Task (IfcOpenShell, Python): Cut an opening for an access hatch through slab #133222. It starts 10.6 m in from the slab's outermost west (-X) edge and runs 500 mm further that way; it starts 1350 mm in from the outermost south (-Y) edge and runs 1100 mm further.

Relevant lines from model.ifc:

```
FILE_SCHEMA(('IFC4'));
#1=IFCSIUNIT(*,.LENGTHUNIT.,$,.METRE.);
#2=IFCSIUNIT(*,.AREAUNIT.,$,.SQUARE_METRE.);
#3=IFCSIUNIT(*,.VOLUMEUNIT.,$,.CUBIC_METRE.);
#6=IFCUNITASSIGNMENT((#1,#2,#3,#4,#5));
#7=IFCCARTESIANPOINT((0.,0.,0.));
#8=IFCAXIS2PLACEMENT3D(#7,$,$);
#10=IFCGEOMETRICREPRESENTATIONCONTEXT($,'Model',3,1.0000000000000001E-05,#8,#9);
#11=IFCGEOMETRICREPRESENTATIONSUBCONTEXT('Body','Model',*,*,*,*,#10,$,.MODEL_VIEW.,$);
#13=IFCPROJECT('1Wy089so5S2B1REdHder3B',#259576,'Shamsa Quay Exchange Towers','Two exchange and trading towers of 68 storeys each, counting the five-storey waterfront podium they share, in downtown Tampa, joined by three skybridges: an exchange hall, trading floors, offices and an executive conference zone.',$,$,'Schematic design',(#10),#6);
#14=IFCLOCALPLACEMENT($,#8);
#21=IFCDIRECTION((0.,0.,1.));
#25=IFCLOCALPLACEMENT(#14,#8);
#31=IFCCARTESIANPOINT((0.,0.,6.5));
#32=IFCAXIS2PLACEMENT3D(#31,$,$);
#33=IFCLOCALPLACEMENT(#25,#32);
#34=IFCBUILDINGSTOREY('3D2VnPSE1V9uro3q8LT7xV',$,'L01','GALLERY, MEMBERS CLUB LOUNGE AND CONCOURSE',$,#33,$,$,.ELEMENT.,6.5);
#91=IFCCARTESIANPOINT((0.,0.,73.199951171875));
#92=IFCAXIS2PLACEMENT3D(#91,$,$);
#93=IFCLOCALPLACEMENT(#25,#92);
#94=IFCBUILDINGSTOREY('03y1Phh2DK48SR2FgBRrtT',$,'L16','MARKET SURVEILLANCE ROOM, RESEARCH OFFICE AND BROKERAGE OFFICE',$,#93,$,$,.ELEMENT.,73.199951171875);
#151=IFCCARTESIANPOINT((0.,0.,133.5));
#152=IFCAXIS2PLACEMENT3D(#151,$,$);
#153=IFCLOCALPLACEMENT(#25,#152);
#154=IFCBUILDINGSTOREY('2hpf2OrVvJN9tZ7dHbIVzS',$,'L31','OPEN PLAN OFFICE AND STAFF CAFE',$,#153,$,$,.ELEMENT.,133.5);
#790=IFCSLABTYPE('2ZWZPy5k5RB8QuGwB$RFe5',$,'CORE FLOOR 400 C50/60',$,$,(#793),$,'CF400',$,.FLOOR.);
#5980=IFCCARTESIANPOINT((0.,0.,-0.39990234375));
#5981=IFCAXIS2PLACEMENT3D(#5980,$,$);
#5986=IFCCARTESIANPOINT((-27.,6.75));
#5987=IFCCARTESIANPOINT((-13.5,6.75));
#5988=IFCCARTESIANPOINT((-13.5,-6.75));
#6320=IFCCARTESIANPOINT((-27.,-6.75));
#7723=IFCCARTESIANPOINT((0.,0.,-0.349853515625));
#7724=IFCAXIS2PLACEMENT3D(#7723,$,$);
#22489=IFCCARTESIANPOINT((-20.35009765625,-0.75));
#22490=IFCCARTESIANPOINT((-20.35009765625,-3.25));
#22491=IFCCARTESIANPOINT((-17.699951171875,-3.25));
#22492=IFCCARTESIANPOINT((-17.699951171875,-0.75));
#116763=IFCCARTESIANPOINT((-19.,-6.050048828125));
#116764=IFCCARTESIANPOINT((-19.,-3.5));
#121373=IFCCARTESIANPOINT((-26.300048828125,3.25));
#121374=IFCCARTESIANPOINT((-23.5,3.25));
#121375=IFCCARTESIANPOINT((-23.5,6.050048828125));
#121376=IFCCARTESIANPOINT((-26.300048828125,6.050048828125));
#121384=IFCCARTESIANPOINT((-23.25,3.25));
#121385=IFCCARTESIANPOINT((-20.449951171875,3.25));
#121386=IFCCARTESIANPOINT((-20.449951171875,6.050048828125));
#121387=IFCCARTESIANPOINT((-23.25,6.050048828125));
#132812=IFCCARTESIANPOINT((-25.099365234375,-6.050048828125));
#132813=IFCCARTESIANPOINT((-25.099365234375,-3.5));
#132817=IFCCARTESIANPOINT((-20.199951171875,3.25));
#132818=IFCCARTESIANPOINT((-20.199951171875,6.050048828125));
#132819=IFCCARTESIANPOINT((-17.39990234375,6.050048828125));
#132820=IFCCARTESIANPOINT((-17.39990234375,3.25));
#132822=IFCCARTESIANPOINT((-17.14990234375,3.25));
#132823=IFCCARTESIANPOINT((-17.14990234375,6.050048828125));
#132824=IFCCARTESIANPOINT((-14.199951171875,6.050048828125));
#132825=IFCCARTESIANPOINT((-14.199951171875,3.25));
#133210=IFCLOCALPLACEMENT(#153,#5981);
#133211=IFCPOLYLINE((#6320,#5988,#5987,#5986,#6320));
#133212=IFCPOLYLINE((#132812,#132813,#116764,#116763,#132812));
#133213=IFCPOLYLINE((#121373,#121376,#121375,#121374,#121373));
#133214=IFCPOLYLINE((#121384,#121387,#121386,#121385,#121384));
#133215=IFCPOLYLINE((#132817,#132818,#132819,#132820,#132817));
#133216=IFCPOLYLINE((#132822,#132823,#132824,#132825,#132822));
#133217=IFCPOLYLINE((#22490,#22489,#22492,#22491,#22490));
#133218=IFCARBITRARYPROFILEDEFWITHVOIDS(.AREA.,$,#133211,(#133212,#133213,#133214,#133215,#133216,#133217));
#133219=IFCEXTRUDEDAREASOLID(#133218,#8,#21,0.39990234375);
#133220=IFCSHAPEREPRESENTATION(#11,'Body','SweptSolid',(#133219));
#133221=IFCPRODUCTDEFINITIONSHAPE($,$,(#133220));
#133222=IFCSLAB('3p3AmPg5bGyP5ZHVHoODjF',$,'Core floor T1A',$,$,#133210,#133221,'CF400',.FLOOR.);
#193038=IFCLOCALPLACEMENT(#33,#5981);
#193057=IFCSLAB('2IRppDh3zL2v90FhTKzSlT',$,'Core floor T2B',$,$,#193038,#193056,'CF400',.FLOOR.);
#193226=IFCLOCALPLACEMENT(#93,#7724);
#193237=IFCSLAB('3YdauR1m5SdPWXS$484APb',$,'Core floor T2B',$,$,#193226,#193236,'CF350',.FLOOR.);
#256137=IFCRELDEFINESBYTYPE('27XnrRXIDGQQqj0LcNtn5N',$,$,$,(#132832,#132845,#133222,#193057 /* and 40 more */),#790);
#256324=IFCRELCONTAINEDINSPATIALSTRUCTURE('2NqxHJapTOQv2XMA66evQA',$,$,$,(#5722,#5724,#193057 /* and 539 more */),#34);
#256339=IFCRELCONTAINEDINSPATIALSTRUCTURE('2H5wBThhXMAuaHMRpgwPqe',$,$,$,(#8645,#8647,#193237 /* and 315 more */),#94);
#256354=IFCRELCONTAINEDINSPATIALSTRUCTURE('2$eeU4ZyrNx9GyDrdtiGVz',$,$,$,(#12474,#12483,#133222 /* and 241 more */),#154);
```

```python
import numpy as np
import ifcopenshell
import ifcopenshell.api.feature
import ifcopenshell.api.geometry
import ifcopenshell.api.root
import ifcopenshell.geom
import ifcopenshell.util.placement
import ifcopenshell.util.representation
import ifcopenshell.util.shape
import ifcopenshell.util.unit

model = ifcopenshell.open("model.ifc")
unit_scale = ifcopenshell.util.unit.calculate_unit_scale(model)
settings = ifcopenshell.geom.settings()


def volume(element):
    """Net volume in cubic metres, openings subtracted."""
    shape = ifcopenshell.geom.create_shape(settings, element)
    return ifcopenshell.util.shape.get_volume(shape.geometry)


slab = model.by_guid("3p3AmPg5bGyP5ZHVHoODjF")
before = volume(slab)

# Extent in the slab's own axes, in metres. The edges named are its -X and -Y sides.
slab_shape = ifcopenshell.geom.create_shape(settings, slab)
vertices = ifcopenshell.util.shape.get_vertices(slab_shape.geometry)
x_min, y_min, bottom = vertices.min(axis=0)
top = vertices[:, 2].max()

opening = ifcopenshell.api.root.create_entity(model, ifc_class="IfcOpeningElement", name="Access hatch opening", predefined_type="OPENING")
context = ifcopenshell.util.representation.get_context(model, "Model", "Body", "MODEL_VIEW")
width, depth = 0.5, 1.1
outline = [(0.0, 0.0), (width, 0.0), (width, depth), (0.0, depth), (0.0, 0.0)]
# Overshoot both faces by 50 mm so the cut is clean.
shape = ifcopenshell.api.geometry.add_slab_representation(
    model, context=context, depth=top - bottom + 0.1, polyline=outline
)
ifcopenshell.api.geometry.assign_representation(model, product=opening, representation=shape)

matrix = ifcopenshell.util.placement.get_local_placement(slab.ObjectPlacement)
matrix[:, 3] = matrix @ np.append(np.array([x_min + 10.6, y_min + 1.35, bottom - 0.05]) / unit_scale, 1.0)
ifcopenshell.api.geometry.edit_object_placement(model, product=opening, matrix=matrix, is_si=False)
ifcopenshell.api.feature.add_feature(model, feature=opening, element=slab)

after = volume(slab)

print(f"slab volume {before:.3f} -> {after:.3f} m3")

model.write("model_v2.ifc")
```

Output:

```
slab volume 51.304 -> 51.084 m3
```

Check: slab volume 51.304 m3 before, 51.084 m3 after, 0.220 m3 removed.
